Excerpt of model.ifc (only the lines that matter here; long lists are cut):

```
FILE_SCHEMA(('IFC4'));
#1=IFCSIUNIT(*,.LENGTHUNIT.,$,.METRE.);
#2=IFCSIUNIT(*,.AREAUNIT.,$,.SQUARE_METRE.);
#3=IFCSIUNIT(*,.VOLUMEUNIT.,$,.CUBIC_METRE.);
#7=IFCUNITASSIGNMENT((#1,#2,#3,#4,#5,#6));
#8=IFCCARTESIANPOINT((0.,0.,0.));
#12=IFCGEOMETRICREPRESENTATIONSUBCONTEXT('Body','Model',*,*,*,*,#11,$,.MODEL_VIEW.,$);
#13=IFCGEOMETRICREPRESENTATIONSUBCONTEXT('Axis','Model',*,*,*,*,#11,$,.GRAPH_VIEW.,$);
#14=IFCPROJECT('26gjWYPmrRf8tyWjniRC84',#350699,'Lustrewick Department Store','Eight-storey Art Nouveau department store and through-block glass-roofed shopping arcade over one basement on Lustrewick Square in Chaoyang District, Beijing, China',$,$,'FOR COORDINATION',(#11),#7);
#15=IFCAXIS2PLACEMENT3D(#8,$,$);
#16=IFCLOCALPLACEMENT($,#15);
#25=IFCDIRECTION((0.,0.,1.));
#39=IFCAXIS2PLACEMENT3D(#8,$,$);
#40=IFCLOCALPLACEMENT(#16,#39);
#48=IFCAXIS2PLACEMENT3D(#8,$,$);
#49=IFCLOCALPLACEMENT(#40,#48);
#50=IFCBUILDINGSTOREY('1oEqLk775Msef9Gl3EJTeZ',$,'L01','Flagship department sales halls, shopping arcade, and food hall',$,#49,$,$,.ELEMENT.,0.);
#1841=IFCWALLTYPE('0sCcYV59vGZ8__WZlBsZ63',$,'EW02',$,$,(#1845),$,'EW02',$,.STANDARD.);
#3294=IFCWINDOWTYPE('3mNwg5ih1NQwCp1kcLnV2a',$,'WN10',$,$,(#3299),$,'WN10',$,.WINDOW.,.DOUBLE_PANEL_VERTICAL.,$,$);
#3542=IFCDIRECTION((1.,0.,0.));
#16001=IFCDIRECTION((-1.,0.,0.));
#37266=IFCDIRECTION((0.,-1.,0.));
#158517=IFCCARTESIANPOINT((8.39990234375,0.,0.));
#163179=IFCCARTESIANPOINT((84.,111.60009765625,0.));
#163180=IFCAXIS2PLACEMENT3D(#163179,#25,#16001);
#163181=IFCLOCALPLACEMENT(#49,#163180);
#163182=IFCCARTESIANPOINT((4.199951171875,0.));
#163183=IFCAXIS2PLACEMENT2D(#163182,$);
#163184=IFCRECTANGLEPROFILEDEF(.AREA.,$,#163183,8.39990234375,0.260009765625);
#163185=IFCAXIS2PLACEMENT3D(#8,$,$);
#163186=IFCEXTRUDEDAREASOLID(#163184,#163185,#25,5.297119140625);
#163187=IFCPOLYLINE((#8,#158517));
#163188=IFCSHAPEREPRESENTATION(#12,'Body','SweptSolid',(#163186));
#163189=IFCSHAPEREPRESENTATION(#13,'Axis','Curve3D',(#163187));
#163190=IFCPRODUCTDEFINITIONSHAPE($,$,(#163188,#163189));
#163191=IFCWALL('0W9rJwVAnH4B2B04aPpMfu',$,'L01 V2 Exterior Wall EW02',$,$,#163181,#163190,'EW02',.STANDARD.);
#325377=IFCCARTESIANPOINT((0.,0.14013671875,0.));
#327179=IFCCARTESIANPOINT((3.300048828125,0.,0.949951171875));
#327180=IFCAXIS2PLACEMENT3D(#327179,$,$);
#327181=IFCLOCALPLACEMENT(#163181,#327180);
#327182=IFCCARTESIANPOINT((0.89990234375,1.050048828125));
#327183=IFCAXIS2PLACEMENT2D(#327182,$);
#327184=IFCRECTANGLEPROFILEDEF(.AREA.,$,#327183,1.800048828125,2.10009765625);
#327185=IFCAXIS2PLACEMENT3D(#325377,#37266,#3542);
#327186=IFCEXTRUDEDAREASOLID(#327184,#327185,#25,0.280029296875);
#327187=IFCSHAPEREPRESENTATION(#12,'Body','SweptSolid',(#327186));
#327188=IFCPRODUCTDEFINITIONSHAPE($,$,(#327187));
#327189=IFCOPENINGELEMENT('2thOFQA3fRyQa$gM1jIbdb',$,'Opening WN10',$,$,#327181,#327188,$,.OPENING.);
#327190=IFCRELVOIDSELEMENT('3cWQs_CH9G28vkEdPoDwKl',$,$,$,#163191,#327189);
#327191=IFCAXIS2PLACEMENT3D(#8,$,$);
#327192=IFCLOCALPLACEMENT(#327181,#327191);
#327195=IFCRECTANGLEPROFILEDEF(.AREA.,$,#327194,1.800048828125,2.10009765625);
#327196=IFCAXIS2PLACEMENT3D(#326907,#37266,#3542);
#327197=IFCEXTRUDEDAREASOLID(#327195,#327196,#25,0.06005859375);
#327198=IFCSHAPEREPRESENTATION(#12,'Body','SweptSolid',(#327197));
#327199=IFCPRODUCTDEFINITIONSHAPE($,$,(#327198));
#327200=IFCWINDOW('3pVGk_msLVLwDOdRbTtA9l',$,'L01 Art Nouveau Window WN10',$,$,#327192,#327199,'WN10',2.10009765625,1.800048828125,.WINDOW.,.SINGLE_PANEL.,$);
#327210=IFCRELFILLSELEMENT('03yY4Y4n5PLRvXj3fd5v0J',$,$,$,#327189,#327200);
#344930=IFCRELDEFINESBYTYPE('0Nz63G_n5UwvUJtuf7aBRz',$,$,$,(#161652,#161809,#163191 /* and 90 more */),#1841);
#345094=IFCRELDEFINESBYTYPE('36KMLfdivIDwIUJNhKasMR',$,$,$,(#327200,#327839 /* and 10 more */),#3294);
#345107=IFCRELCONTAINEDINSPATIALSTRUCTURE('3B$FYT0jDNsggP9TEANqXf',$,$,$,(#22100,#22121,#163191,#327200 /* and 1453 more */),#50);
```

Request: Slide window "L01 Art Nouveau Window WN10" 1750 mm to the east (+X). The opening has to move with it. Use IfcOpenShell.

```python
import ifcopenshell
import ifcopenshell.api.geometry
import ifcopenshell.util.placement

model = ifcopenshell.open("model.ifc")

window = model.by_guid("3pVGk_msLVLwDOdRbTtA9l")
opening = window.FillsVoids[0].RelatingOpeningElement
wall = opening.VoidsElements[0].RelatingBuildingElement

wall_matrix = ifcopenshell.util.placement.get_local_placement(wall.ObjectPlacement)
shift = wall_matrix[:3, 0] * -1.75
before = ifcopenshell.util.placement.get_local_placement(window.ObjectPlacement)[:3, 3].copy()

# The window is placed relative to its opening, so it follows when the opening moves.
matrix = ifcopenshell.util.placement.get_local_placement(opening.ObjectPlacement)
matrix[:3, 3] += shift
ifcopenshell.api.geometry.edit_object_placement(
    model, product=opening, matrix=matrix, is_si=False, should_transform_children=True
)

after = ifcopenshell.util.placement.get_local_placement(window.ObjectPlacement)[:3, 3]
print("window moved by", (after - before).round(3) + 0.0)

model.write("model_v2.ifc")
```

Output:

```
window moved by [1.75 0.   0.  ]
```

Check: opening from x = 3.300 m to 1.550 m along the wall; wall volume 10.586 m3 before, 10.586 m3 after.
